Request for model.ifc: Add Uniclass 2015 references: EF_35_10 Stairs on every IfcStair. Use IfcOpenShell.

First a look at what the model holds.

```python
import ifcopenshell

model = ifcopenshell.open("model.ifc")
print(model.schema)
print("classifications:", [c.Name for c in model.by_type("IfcClassification")])
for ifc_class in ("IfcDoor", "IfcRoof", "IfcStair", "IfcWall", "IfcWindow"):
    print(ifc_class, len(model.by_type(ifc_class)))
```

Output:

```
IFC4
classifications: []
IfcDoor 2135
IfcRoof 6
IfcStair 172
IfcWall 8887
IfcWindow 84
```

```python
import ifcopenshell
import ifcopenshell.api.classification

model = ifcopenshell.open("model.ifc")

system = ifcopenshell.api.classification.add_classification(model, classification="Uniclass 2015")

codes = {
    "IfcStair": ("EF_35_10", "Stairs"),
}
for ifc_class, (code, name) in codes.items():
    products = model.by_type(ifc_class)
    ifcopenshell.api.classification.add_reference(
        model, products=products, classification=system, identification=code, name=name
    )
    print(code, len(products))

model.write("model_v2.ifc")
```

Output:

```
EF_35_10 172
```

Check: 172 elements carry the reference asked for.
